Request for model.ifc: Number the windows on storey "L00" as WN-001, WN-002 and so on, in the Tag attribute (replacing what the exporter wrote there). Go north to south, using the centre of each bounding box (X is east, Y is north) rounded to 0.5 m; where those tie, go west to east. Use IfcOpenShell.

First a look at what the model holds.

```python
import ifcopenshell
import ifcopenshell.util.element
import ifcopenshell.util.placement

model = ifcopenshell.open("model.ifc")
print(model.schema)
storey = next(s for s in model.by_type("IfcBuildingStorey") if s.Name == "L00")
windows = [e for e in ifcopenshell.util.element.get_decomposition(storey) if e.is_a("IfcWindow")]
for e in sorted(windows, key=lambda e: e.id()):
    origin = ifcopenshell.util.placement.get_local_placement(e.ObjectPlacement)[:3, 3]
    print(e.id(), e.Tag, e.Name, origin.round(2) + 0.0, sep=" | ")
```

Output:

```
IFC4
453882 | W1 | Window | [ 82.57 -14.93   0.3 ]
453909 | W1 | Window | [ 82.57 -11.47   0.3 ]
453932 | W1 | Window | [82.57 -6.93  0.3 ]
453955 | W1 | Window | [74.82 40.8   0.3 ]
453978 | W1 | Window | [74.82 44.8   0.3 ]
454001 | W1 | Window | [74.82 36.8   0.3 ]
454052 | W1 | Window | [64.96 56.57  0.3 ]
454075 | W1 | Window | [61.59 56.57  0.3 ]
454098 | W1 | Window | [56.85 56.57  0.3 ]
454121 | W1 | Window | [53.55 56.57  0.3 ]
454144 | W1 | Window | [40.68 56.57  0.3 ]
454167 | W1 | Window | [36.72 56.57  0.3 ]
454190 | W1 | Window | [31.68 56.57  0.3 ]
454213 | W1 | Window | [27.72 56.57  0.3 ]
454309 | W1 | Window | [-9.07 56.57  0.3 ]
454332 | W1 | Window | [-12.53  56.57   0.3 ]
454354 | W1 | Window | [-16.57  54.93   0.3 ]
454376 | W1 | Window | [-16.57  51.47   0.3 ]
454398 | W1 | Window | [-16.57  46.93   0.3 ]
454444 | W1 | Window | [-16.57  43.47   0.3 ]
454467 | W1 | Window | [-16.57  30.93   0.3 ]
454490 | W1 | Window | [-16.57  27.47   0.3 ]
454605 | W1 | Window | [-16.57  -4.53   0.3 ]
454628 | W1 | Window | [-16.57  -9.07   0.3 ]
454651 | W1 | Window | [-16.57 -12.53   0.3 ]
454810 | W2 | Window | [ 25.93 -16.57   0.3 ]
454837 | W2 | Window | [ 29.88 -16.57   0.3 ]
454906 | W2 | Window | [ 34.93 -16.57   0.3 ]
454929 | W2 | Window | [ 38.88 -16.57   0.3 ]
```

```python
import ifcopenshell
import ifcopenshell.geom
import ifcopenshell.util.element
import ifcopenshell.util.shape

model = ifcopenshell.open("model.ifc")
settings = ifcopenshell.geom.settings()
settings.set("use-world-coords", True)


def centre(element):
    shape = ifcopenshell.geom.create_shape(settings, element)
    return ifcopenshell.util.shape.get_bbox_centroid(shape.geometry)


storey = next(s for s in model.by_type("IfcBuildingStorey") if s.Name == "L00")
windows = [e for e in ifcopenshell.util.element.get_decomposition(storey) if e.is_a("IfcWindow")]

# Insertion points can sit at a corner or the storey origin, so sort by the geometry (in metres).
centres = {e: centre(e) for e in windows}
windows.sort(key=lambda e: (-round(centres[e][1] / 0.5), centres[e][0]))

for i, e in enumerate(windows, start=1):
    number = f"WN-0{i:02d}"
    e.Tag = number
    print(e.id(), number)

model.write("model-out.ifc")
```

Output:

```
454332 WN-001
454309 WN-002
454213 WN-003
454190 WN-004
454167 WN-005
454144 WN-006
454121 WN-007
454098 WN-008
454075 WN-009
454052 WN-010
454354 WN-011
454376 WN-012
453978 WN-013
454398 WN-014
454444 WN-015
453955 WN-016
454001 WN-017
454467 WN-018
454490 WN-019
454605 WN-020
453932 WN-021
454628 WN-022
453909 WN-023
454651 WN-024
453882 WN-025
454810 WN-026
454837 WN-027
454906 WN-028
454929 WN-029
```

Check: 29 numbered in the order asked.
